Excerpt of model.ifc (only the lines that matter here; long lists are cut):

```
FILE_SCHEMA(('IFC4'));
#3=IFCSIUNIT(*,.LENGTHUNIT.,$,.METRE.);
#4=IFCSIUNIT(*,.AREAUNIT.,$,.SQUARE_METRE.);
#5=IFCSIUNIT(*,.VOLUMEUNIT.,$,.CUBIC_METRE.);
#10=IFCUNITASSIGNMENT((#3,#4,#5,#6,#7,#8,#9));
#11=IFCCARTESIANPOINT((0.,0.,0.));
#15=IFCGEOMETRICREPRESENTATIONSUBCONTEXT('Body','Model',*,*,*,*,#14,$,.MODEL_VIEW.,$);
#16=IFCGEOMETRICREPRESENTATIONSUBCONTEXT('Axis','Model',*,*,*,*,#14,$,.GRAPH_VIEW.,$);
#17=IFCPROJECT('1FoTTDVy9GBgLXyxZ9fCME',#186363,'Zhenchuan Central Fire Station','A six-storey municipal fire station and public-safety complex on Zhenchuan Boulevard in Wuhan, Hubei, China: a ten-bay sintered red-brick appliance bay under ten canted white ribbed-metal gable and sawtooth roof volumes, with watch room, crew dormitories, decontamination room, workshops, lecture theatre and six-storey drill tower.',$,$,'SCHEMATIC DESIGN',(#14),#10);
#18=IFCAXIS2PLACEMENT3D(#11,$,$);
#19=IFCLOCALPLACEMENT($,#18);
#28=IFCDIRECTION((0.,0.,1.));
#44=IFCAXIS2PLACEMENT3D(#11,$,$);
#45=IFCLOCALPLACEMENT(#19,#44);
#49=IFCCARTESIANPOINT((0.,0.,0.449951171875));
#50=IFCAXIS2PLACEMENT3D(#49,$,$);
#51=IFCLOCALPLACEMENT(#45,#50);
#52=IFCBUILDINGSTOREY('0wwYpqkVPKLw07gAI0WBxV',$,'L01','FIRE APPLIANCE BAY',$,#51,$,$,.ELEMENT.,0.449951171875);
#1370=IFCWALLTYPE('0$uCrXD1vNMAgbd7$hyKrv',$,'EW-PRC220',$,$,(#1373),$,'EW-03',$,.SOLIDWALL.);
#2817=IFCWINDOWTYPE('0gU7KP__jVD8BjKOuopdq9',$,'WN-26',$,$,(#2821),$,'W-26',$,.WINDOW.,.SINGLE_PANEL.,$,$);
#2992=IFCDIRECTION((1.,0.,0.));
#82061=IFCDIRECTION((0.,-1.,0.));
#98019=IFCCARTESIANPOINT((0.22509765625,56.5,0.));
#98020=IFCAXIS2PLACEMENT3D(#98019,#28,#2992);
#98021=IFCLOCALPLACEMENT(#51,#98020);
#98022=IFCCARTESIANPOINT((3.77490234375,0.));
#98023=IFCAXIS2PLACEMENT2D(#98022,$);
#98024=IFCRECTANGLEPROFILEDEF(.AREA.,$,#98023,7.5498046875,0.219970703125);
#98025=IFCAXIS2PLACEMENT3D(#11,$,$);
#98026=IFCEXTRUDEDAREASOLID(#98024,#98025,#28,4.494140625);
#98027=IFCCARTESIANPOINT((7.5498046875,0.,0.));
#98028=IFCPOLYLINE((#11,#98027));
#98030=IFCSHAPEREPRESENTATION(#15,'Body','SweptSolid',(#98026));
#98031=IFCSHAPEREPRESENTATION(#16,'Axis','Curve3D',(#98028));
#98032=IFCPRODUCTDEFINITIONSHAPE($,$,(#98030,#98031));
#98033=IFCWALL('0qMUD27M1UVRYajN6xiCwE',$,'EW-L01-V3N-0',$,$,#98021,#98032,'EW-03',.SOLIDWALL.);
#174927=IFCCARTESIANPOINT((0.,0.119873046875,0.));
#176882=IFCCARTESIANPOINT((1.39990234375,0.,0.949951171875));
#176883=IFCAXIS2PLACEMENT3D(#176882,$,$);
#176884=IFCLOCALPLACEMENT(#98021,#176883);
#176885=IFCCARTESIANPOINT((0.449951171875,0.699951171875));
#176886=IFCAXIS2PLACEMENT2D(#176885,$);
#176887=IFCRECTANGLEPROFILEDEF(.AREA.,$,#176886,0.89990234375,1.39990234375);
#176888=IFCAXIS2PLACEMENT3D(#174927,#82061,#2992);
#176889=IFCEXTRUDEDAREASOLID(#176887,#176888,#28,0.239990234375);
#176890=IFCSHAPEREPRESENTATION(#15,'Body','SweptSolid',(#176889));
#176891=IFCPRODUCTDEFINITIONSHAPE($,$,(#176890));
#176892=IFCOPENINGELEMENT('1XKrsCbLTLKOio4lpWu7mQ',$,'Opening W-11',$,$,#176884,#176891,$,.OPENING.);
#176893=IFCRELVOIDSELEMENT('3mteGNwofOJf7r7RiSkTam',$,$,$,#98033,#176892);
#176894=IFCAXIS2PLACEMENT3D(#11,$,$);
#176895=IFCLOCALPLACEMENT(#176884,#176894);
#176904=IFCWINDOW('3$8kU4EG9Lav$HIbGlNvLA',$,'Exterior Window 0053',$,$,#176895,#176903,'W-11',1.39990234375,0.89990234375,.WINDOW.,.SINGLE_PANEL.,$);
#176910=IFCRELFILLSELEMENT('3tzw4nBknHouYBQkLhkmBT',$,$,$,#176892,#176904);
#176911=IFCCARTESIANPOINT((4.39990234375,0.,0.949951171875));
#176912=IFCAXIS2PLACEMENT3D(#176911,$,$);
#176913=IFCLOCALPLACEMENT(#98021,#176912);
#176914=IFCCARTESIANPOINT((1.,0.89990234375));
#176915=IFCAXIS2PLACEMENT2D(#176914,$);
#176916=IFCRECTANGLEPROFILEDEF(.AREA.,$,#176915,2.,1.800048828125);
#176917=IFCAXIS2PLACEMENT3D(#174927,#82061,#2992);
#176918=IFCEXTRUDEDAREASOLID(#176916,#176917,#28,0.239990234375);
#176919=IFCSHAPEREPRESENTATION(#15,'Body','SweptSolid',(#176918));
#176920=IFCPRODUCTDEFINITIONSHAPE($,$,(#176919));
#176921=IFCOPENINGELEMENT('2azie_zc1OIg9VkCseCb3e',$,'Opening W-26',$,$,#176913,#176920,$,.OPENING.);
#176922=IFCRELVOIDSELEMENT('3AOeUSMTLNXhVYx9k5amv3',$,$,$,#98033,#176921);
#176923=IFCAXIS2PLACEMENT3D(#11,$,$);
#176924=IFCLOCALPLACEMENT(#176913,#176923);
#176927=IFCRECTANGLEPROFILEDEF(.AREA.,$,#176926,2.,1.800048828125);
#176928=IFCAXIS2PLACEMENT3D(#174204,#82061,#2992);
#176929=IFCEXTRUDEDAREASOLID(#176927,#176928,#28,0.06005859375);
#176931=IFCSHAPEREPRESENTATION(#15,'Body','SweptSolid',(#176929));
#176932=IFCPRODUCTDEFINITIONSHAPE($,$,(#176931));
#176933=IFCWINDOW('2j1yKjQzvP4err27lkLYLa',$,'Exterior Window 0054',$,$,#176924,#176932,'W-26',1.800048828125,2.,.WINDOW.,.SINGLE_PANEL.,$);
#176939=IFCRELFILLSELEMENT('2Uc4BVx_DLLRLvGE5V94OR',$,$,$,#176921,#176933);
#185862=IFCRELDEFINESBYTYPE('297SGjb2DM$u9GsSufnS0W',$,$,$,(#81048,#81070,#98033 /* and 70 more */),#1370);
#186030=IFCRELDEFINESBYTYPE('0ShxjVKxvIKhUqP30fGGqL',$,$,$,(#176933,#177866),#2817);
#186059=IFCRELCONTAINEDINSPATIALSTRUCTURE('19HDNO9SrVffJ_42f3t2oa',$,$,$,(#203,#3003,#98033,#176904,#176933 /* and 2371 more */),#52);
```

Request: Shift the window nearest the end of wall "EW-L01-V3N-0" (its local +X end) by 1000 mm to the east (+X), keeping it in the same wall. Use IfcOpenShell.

```python
import ifcopenshell
import ifcopenshell.api.geometry
import ifcopenshell.util.placement
import ifcopenshell.util.unit

model = ifcopenshell.open("model.ifc")
unit_scale = ifcopenshell.util.unit.calculate_unit_scale(model)

window = model.by_guid("2j1yKjQzvP4err27lkLYLa")
opening = window.FillsVoids[0].RelatingOpeningElement
wall = opening.VoidsElements[0].RelatingBuildingElement

wall_matrix = ifcopenshell.util.placement.get_local_placement(wall.ObjectPlacement)
shift = wall_matrix[:3, 0] * 1 / unit_scale
before = ifcopenshell.util.placement.get_local_placement(window.ObjectPlacement)[:3, 3].copy()

# The window is placed relative to its opening, so it follows when the opening moves.
matrix = ifcopenshell.util.placement.get_local_placement(opening.ObjectPlacement)
matrix[:3, 3] += shift
ifcopenshell.api.geometry.edit_object_placement(
    model, product=opening, matrix=matrix, is_si=False, should_transform_children=True
)

after = ifcopenshell.util.placement.get_local_placement(window.ObjectPlacement)[:3, 3]
print("window moved by", (after - before).round(3) + 0.0)

model.write("model_edited.ifc")
```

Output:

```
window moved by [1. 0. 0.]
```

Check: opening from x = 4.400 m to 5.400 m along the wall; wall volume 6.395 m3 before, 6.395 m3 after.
